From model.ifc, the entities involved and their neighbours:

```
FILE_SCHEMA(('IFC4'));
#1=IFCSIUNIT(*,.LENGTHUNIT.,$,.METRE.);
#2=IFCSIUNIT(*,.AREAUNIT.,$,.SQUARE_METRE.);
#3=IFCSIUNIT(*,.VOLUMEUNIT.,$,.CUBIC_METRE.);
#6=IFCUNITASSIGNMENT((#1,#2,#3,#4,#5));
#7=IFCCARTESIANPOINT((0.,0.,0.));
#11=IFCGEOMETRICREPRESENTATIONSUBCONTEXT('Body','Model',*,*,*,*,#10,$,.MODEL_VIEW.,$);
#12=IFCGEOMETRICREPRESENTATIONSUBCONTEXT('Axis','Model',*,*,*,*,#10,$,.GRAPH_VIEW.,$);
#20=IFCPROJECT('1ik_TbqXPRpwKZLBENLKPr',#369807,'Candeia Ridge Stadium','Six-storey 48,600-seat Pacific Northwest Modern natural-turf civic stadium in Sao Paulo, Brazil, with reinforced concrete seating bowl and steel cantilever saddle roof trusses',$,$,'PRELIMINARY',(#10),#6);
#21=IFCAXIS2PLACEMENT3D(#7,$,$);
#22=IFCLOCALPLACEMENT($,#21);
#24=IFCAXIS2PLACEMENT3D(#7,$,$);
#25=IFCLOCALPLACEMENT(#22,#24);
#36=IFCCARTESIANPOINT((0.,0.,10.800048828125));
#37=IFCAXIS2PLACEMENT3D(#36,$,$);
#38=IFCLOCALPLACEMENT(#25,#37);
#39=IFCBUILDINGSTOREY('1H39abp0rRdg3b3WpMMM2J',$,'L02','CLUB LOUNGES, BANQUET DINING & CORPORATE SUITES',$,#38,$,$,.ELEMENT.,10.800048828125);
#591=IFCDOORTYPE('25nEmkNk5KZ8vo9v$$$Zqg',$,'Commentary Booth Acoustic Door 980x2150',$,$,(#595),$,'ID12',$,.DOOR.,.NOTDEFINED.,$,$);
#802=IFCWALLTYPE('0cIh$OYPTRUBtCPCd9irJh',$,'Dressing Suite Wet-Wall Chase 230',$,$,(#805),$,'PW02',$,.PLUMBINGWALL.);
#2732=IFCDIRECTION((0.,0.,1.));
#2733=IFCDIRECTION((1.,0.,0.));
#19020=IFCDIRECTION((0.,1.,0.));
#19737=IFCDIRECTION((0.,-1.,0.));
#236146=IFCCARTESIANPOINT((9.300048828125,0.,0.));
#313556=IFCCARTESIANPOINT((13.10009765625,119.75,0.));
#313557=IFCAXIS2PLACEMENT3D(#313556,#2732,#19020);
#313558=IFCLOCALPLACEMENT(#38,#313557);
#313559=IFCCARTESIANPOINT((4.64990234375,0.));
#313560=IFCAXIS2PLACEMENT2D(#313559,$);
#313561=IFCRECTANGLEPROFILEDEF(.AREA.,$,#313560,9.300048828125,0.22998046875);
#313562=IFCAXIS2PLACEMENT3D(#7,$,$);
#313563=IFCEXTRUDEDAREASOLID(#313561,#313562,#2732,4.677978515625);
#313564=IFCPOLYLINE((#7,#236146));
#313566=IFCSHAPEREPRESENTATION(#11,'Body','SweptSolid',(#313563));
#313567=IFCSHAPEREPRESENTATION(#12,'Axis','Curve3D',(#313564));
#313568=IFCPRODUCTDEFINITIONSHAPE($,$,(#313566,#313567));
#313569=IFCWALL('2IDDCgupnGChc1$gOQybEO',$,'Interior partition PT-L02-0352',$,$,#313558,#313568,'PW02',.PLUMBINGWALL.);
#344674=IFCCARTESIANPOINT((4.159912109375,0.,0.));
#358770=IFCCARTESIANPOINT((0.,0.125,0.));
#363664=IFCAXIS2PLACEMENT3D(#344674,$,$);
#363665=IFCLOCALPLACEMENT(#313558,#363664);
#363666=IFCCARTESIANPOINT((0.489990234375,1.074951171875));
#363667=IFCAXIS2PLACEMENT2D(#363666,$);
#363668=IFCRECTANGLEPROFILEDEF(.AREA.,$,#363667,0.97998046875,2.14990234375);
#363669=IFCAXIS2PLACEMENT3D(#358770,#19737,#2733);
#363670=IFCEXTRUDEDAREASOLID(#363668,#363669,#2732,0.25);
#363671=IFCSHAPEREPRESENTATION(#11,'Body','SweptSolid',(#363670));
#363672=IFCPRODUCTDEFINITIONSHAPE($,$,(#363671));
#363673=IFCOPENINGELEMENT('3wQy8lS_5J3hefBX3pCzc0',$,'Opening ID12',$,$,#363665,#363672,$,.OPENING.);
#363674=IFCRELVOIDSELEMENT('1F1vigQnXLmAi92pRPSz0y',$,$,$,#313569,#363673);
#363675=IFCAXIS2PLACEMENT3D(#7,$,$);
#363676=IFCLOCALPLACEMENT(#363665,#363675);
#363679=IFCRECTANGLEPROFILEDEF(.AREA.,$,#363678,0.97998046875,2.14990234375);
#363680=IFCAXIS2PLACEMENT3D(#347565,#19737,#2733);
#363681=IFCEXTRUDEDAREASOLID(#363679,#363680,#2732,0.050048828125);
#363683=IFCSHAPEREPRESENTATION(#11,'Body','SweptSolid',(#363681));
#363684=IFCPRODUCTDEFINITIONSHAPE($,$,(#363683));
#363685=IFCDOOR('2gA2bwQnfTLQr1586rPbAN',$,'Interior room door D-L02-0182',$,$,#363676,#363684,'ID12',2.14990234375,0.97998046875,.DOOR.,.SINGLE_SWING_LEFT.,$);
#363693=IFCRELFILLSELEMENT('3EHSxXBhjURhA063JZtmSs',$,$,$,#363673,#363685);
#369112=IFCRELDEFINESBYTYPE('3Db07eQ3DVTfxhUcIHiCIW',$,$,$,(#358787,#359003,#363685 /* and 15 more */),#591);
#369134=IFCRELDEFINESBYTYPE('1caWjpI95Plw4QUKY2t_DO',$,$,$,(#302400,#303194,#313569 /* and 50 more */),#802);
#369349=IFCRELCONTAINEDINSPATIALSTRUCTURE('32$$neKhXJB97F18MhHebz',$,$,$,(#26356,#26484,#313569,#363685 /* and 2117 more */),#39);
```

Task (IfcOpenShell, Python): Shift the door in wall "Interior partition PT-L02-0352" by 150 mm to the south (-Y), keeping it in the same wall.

```python
import ifcopenshell
import ifcopenshell.api.geometry
import ifcopenshell.util.placement

model = ifcopenshell.open("model.ifc")

door = model.by_id(363685)
opening = door.FillsVoids[0].RelatingOpeningElement
wall = opening.VoidsElements[0].RelatingBuildingElement

wall_matrix = ifcopenshell.util.placement.get_local_placement(wall.ObjectPlacement)
shift = wall_matrix[:3, 0] * -0.15
before = ifcopenshell.util.placement.get_local_placement(door.ObjectPlacement)[:3, 3].copy()

# The door is placed relative to its opening, so it follows when the opening moves.
matrix = ifcopenshell.util.placement.get_local_placement(opening.ObjectPlacement)
matrix[:3, 3] += shift
ifcopenshell.api.geometry.edit_object_placement(
    model, product=opening, matrix=matrix, is_si=False, should_transform_children=True
)

after = ifcopenshell.util.placement.get_local_placement(door.ObjectPlacement)[:3, 3]
print("door moved by", (after - before).round(3) + 0.0)

model.write("model_edited.ifc")
```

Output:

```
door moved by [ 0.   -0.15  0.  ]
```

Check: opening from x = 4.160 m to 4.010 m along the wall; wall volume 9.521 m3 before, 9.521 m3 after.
